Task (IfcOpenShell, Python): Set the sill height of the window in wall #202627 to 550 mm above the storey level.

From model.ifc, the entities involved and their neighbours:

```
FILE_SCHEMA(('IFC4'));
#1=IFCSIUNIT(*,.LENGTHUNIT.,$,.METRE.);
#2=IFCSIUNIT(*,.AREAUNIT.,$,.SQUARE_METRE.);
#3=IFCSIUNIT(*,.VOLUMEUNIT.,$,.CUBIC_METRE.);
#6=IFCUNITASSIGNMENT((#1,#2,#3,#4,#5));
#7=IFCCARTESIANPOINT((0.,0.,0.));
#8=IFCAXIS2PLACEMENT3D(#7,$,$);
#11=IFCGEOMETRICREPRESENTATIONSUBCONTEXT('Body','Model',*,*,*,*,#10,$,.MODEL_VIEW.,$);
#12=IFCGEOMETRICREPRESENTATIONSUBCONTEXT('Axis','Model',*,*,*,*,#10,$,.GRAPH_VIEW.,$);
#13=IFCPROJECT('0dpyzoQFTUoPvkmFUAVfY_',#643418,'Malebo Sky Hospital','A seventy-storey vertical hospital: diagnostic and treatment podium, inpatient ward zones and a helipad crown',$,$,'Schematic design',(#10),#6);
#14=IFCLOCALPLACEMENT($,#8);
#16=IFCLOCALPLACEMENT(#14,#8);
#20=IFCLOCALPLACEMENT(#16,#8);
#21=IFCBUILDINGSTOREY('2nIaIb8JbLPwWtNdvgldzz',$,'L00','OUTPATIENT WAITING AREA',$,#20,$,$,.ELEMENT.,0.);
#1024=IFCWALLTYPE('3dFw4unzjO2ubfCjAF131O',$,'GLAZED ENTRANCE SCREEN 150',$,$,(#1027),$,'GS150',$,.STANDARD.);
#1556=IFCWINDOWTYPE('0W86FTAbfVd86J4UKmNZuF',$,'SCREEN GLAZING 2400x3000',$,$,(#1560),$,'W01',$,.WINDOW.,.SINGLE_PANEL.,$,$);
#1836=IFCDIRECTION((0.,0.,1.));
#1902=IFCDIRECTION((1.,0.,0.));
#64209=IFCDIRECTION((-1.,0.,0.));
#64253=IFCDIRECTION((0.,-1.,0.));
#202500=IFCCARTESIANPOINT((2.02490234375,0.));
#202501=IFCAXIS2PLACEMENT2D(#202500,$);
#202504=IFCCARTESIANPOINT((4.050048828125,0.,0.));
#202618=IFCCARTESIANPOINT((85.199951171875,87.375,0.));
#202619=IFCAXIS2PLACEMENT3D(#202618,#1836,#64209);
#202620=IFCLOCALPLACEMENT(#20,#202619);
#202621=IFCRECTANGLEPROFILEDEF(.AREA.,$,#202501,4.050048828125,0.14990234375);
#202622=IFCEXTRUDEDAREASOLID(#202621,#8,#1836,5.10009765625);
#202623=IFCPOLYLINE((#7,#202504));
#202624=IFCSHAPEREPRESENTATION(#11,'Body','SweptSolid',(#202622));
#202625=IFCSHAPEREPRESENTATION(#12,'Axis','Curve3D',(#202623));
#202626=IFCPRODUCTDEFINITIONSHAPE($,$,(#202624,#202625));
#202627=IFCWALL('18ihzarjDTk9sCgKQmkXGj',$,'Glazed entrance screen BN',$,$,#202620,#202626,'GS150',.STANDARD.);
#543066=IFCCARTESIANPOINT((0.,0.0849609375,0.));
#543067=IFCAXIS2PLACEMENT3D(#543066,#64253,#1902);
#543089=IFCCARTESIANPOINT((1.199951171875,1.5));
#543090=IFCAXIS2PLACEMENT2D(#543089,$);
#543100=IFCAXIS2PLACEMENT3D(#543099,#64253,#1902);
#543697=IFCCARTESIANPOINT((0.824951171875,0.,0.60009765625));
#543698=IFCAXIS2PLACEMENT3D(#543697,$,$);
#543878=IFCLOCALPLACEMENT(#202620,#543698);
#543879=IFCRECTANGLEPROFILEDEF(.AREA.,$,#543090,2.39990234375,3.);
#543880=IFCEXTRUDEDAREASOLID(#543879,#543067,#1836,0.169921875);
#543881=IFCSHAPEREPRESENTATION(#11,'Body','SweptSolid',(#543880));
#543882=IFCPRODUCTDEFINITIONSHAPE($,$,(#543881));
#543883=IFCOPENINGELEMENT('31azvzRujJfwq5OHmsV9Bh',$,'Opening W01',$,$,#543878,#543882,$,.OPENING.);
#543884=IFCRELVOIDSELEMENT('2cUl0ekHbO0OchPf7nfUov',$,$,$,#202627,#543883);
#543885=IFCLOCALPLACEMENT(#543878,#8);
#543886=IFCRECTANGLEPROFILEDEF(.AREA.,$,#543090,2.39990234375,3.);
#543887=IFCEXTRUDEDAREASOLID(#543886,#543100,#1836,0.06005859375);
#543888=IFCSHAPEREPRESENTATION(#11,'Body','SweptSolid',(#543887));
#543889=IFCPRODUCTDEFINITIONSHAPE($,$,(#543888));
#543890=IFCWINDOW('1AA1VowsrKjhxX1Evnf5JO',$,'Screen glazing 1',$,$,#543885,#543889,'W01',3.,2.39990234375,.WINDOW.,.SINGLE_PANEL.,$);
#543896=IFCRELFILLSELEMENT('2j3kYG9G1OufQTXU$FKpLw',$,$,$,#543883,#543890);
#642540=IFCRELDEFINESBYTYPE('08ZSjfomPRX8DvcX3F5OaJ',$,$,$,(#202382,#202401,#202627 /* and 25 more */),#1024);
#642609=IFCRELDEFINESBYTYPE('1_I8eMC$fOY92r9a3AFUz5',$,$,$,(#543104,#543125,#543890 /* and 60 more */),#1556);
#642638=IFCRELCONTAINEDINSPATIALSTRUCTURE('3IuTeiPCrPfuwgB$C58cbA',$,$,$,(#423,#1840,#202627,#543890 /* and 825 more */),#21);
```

```python
import numpy as np
import ifcopenshell
import ifcopenshell.api.geometry
import ifcopenshell.geom
import ifcopenshell.util.element
import ifcopenshell.util.placement
import ifcopenshell.util.shape
import ifcopenshell.util.unit

model = ifcopenshell.open("model.ifc")
unit_scale = ifcopenshell.util.unit.calculate_unit_scale(model)

window = model.by_guid("1AA1VowsrKjhxX1Evnf5JO")
opening = window.FillsVoids[0].RelatingOpeningElement
storey = ifcopenshell.util.element.get_container(window, ifc_class="IfcBuildingStorey")
level = ifcopenshell.util.placement.get_local_placement(storey.ObjectPlacement)[2, 3]

# The opening's origin need not be at the sill, so measure its lowest point.
shape = ifcopenshell.geom.create_shape(ifcopenshell.geom.settings(), opening)
bottom = ifcopenshell.util.shape.get_shape_bottom_elevation(shape, shape.geometry) / unit_scale
dz = level + 0.55 / unit_scale - bottom

shift = np.array([0.0, 0.0, dz])
# The window is placed relative to its opening, so it follows when the opening moves.
matrix = ifcopenshell.util.placement.get_local_placement(opening.ObjectPlacement)
matrix[:3, 3] += shift
ifcopenshell.api.geometry.edit_object_placement(
    model, product=opening, matrix=matrix, is_si=False, should_transform_children=True
)

print(f"moved by {dz * unit_scale:+.3f} m")

model.write("model_rev.ifc")
```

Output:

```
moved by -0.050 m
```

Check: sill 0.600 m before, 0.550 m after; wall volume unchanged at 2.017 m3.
